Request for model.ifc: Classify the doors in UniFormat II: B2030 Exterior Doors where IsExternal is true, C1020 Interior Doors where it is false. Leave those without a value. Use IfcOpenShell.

First a look at what the model holds.

```python
import ifcopenshell
import ifcopenshell.util.element

model = ifcopenshell.open("model.ifc")
print(model.schema)
print("classifications:", [c.Name for c in model.by_type("IfcClassification")])
values = [ifcopenshell.util.element.get_pset(e, "Pset_DoorCommon", "IsExternal") for e in model.by_type("IfcDoor")]
for value in (True, False, None):
    print("IsExternal", value, values.count(value))
```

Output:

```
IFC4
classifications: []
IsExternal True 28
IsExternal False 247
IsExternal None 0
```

```python
import ifcopenshell
import ifcopenshell.api.classification
import ifcopenshell.util.element

model = ifcopenshell.open("model.ifc")

system = ifcopenshell.api.classification.add_classification(model, classification="UniFormat II")

doors = model.by_type("IfcDoor")
external = {e: ifcopenshell.util.element.get_pset(e, "Pset_DoorCommon", "IsExternal") for e in doors}
for flag, code, name in ((True, "B2030", "Exterior Doors"), (False, "C1020", "Interior Doors")):
    products = [e for e in doors if external[e] is flag]
    ifcopenshell.api.classification.add_reference(
        model, products=products, classification=system, identification=code, name=name
    )
    print(code, len(products))

model.write("model_edited.ifc")
```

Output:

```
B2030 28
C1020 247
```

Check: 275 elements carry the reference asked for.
